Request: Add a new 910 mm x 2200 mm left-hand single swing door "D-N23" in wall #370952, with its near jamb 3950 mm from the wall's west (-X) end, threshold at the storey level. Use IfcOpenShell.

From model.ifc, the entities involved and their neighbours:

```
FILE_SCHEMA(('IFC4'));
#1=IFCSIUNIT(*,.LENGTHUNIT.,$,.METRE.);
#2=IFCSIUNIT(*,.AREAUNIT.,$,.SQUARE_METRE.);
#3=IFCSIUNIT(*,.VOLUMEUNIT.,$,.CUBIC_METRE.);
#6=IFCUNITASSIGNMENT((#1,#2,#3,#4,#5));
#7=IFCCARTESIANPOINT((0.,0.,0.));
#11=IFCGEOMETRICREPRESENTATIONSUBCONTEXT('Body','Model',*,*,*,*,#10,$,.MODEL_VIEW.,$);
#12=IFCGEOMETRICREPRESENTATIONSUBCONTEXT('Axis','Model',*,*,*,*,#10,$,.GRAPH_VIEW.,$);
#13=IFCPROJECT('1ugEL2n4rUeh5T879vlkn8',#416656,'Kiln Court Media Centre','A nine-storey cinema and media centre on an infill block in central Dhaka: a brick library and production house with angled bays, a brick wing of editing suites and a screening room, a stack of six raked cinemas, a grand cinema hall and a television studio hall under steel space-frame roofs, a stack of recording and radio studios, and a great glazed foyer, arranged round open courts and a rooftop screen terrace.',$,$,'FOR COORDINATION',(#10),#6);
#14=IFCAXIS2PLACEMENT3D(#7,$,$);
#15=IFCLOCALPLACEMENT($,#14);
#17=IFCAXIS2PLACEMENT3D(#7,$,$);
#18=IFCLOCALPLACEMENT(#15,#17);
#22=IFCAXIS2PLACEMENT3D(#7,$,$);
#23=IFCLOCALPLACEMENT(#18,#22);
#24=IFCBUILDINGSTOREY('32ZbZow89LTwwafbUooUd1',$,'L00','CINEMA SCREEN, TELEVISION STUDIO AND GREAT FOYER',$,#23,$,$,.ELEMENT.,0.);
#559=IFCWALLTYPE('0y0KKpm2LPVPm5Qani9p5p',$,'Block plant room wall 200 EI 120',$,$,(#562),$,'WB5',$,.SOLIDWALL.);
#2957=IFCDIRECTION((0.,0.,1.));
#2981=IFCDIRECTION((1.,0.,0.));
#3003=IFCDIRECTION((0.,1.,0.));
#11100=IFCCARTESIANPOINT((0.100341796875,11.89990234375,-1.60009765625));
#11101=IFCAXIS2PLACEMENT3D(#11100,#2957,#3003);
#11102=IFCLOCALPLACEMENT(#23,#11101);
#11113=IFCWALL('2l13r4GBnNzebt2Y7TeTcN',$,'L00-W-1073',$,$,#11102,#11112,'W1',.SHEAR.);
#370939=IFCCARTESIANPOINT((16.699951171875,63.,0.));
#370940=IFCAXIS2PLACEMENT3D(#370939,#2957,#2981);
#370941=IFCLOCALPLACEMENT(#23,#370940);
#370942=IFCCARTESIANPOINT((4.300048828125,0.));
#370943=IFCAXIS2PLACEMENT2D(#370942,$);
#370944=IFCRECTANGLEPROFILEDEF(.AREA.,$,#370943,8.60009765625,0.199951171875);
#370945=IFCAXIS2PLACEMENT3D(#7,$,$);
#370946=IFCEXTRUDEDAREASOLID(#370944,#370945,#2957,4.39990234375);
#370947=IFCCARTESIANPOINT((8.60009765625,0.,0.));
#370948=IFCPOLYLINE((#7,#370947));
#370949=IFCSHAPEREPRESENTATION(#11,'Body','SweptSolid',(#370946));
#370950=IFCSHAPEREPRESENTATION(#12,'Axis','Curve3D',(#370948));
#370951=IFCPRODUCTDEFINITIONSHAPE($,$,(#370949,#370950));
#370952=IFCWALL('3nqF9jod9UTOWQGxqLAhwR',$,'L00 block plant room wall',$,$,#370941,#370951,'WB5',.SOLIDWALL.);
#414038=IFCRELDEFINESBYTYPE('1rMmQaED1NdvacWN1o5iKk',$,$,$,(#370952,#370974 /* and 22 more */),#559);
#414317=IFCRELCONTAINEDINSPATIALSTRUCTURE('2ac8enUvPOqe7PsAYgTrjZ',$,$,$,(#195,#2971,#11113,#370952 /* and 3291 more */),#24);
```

```python
import numpy as np
import ifcopenshell
import ifcopenshell.api.feature
import ifcopenshell.api.geometry
import ifcopenshell.api.root
import ifcopenshell.api.spatial
import ifcopenshell.geom
import ifcopenshell.util.element
import ifcopenshell.util.placement
import ifcopenshell.util.representation
import ifcopenshell.util.shape
import ifcopenshell.util.unit

model = ifcopenshell.open("model.ifc")
unit_scale = ifcopenshell.util.unit.calculate_unit_scale(model)
settings = ifcopenshell.geom.settings()


def volume(element):
    """Net volume in cubic metres, openings subtracted."""
    shape = ifcopenshell.geom.create_shape(settings, element)
    return ifcopenshell.util.shape.get_volume(shape.geometry)


wall = model.by_guid("3nqF9jod9UTOWQGxqLAhwR")
storey = ifcopenshell.util.element.get_container(wall, ifc_class="IfcBuildingStorey")
context = ifcopenshell.util.representation.get_context(model, "Model", "Body", "MODEL_VIEW")
before = volume(wall)

width, height, from_end, sill = 0.91, 2.2, 3.95, 0.0  # metres

# The wall runs along its own X axis, and the end named is its -X end.
wall_shape = ifcopenshell.geom.create_shape(settings, wall)
x, y, z = ifcopenshell.util.shape.get_vertices(wall_shape.geometry).T
start = x.min() + from_end
face, thickness = float(y.min()), float(y.max() - y.min())
wall_matrix = ifcopenshell.util.placement.get_local_placement(wall.ObjectPlacement)
level = ifcopenshell.util.placement.get_local_placement(storey.ObjectPlacement)[2, 3]


def in_wall(x, y):
    """Placement at x, y metres in the wall's axes, at sill height."""
    matrix = wall_matrix.copy()
    matrix[:, 3] = wall_matrix @ np.array([x / unit_scale, y / unit_scale, 0.0, 1.0])
    matrix[2, 3] = level + sill / unit_scale
    return matrix


# Opening: a box that overshoots both wall faces by 50 mm.
opening = ifcopenshell.api.root.create_entity(model, ifc_class="IfcOpeningElement", predefined_type="OPENING")
box = ifcopenshell.api.geometry.add_wall_representation(
    model, context=context, length=width, height=height, thickness=thickness + 0.1
)
ifcopenshell.api.geometry.assign_representation(model, product=opening, representation=box)
ifcopenshell.api.geometry.edit_object_placement(model, product=opening, matrix=in_wall(start, face - 0.05), is_si=False)
ifcopenshell.api.feature.add_feature(model, feature=opening, element=wall)

door = ifcopenshell.api.root.create_entity(model, ifc_class="IfcDoor", name="D-N23", predefined_type="DOOR")
door.OverallWidth, door.OverallHeight = width / unit_scale, height / unit_scale
door.OperationType = "SINGLE_SWING_LEFT"
body = ifcopenshell.api.geometry.add_door_representation(
    model,
    context=context,
    overall_width=door.OverallWidth,
    overall_height=door.OverallHeight,
    operation_type="SINGLE_SWING_LEFT",
    lining_properties={"LiningDepth": thickness / unit_scale, "ThresholdDepth": thickness / unit_scale},
)
ifcopenshell.api.geometry.assign_representation(model, product=door, representation=body)
ifcopenshell.api.spatial.assign_container(model, products=[door], relating_structure=storey)
ifcopenshell.api.feature.add_filling(model, opening=opening, element=door)

# The lining spans the wall, so the door starts at the wall face.
ifcopenshell.api.geometry.edit_object_placement(model, product=door, matrix=in_wall(start, face), is_si=False)

after = volume(wall)

print(f"wall volume {before:.3f} -> {after:.3f} m3")

model.write("model-out.ifc")
```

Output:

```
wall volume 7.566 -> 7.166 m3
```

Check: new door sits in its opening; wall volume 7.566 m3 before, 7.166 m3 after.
